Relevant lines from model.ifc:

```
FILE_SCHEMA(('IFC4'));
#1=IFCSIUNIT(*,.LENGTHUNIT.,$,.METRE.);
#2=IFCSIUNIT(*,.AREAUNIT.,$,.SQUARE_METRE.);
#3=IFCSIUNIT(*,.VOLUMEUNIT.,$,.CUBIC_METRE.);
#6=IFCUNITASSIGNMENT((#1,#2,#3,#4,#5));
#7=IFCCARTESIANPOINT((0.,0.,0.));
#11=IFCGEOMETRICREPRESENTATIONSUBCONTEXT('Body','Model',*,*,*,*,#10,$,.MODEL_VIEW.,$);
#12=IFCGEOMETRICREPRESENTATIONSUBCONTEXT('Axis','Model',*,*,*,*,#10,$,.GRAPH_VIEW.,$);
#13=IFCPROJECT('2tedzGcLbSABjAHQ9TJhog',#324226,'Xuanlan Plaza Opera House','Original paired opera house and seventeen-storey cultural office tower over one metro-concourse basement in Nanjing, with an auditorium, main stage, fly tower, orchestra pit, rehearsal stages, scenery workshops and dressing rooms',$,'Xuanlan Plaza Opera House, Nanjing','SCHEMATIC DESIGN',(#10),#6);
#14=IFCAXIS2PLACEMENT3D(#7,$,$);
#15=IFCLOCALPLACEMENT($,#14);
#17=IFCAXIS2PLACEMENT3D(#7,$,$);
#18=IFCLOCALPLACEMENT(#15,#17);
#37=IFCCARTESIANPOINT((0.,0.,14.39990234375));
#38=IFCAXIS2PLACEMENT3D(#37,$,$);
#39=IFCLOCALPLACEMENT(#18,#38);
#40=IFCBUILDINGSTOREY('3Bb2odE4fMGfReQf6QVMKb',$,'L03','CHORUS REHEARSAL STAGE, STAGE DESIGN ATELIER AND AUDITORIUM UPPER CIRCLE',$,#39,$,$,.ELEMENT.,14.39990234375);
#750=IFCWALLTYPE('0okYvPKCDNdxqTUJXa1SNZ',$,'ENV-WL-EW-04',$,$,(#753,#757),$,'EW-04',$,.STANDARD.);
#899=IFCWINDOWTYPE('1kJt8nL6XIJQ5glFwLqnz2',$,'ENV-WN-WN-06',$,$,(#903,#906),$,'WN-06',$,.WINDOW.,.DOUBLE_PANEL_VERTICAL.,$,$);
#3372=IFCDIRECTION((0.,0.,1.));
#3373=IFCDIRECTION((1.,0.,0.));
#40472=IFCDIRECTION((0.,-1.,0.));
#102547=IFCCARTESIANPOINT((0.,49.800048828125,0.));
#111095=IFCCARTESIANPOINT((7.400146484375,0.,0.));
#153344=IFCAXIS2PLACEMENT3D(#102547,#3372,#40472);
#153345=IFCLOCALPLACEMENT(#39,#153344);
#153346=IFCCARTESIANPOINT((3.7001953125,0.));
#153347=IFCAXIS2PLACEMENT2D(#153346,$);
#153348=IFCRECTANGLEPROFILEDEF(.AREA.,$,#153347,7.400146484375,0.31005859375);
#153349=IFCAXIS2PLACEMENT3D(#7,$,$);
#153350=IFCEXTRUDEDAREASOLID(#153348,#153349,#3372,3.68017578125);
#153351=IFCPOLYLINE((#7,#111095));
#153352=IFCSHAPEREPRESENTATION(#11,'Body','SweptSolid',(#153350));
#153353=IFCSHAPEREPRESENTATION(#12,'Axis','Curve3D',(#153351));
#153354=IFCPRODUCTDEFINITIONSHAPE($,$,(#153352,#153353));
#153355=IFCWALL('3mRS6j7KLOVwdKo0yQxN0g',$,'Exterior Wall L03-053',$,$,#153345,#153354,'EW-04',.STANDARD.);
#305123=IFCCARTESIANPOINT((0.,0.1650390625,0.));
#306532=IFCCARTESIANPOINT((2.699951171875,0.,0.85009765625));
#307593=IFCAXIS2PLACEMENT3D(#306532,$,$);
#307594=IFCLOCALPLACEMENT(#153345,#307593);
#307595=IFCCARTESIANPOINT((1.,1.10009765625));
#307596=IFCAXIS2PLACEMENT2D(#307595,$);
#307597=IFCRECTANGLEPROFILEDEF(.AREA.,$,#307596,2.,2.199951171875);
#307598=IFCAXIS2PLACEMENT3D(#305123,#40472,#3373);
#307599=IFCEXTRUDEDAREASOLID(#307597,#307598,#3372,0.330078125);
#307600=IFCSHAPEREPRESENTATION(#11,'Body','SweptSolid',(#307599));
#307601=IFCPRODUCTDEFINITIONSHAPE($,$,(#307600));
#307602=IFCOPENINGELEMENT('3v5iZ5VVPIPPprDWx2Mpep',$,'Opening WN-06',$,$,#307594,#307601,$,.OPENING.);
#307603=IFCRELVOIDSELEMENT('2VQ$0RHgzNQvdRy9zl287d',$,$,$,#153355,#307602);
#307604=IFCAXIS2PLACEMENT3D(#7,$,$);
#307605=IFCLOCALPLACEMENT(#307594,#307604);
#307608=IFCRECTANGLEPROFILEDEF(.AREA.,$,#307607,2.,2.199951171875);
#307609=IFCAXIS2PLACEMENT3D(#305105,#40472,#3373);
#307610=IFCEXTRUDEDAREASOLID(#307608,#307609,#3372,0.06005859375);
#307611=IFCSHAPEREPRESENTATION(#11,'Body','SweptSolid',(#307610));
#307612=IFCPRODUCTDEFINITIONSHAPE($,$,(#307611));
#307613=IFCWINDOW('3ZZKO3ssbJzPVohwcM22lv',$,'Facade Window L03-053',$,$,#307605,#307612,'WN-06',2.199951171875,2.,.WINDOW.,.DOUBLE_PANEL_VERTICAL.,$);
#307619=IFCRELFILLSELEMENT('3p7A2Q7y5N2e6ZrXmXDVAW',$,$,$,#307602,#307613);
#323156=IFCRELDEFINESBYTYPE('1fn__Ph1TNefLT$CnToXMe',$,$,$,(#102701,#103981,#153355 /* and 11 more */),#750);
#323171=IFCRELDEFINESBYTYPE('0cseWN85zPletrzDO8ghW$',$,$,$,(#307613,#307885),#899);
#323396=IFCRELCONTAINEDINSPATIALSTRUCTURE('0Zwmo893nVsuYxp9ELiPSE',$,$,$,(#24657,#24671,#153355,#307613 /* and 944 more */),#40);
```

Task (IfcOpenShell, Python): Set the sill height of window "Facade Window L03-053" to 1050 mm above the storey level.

```python
import numpy as np
import ifcopenshell
import ifcopenshell.api.geometry
import ifcopenshell.geom
import ifcopenshell.util.element
import ifcopenshell.util.placement
import ifcopenshell.util.shape
import ifcopenshell.util.unit

model = ifcopenshell.open("model.ifc")
unit_scale = ifcopenshell.util.unit.calculate_unit_scale(model)

window = model.by_guid("3ZZKO3ssbJzPVohwcM22lv")
opening = window.FillsVoids[0].RelatingOpeningElement
storey = ifcopenshell.util.element.get_container(window, ifc_class="IfcBuildingStorey")
level = ifcopenshell.util.placement.get_local_placement(storey.ObjectPlacement)[2, 3]

# The opening's origin need not be at the sill, so measure its lowest point.
shape = ifcopenshell.geom.create_shape(ifcopenshell.geom.settings(), opening)
bottom = ifcopenshell.util.shape.get_shape_bottom_elevation(shape, shape.geometry) / unit_scale
dz = level + 1.05 / unit_scale - bottom

shift = np.array([0.0, 0.0, dz])
# The window is placed relative to its opening, so it follows when the opening moves.
matrix = ifcopenshell.util.placement.get_local_placement(opening.ObjectPlacement)
matrix[:3, 3] += shift
ifcopenshell.api.geometry.edit_object_placement(
    model, product=opening, matrix=matrix, is_si=False, should_transform_children=True
)

print(f"moved by {dz * unit_scale:+.3f} m")

model.write("model_v2.ifc")
```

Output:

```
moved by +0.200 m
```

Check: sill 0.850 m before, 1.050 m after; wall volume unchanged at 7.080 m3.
